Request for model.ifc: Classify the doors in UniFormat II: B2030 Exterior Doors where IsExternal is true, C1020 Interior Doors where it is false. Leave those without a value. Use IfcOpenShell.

First a look at what the model holds.

```python
import ifcopenshell
import ifcopenshell.util.element

model = ifcopenshell.open("model.ifc")
print(model.schema)
print("classifications:", [c.Name for c in model.by_type("IfcClassification")])
values = [ifcopenshell.util.element.get_pset(e, "Pset_DoorCommon", "IsExternal") for e in model.by_type("IfcDoor")]
for value in (True, False, None):
    print("IsExternal", value, values.count(value))
```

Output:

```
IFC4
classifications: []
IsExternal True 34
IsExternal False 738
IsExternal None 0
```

```python
import ifcopenshell
import ifcopenshell.api.classification
import ifcopenshell.util.element

model = ifcopenshell.open("model.ifc")

system = ifcopenshell.api.classification.add_classification(model, classification="UniFormat II")

doors = model.by_type("IfcDoor")
external = {e: ifcopenshell.util.element.get_pset(e, "Pset_DoorCommon", "IsExternal") for e in doors}
for flag, code, name in ((True, "B2030", "Exterior Doors"), (False, "C1020", "Interior Doors")):
    products = [e for e in doors if external[e] is flag]
    ifcopenshell.api.classification.add_reference(
        model, products=products, classification=system, identification=code, name=name
    )
    print(code, len(products))

model.write("model_updated.ifc")
```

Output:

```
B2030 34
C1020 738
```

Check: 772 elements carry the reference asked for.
